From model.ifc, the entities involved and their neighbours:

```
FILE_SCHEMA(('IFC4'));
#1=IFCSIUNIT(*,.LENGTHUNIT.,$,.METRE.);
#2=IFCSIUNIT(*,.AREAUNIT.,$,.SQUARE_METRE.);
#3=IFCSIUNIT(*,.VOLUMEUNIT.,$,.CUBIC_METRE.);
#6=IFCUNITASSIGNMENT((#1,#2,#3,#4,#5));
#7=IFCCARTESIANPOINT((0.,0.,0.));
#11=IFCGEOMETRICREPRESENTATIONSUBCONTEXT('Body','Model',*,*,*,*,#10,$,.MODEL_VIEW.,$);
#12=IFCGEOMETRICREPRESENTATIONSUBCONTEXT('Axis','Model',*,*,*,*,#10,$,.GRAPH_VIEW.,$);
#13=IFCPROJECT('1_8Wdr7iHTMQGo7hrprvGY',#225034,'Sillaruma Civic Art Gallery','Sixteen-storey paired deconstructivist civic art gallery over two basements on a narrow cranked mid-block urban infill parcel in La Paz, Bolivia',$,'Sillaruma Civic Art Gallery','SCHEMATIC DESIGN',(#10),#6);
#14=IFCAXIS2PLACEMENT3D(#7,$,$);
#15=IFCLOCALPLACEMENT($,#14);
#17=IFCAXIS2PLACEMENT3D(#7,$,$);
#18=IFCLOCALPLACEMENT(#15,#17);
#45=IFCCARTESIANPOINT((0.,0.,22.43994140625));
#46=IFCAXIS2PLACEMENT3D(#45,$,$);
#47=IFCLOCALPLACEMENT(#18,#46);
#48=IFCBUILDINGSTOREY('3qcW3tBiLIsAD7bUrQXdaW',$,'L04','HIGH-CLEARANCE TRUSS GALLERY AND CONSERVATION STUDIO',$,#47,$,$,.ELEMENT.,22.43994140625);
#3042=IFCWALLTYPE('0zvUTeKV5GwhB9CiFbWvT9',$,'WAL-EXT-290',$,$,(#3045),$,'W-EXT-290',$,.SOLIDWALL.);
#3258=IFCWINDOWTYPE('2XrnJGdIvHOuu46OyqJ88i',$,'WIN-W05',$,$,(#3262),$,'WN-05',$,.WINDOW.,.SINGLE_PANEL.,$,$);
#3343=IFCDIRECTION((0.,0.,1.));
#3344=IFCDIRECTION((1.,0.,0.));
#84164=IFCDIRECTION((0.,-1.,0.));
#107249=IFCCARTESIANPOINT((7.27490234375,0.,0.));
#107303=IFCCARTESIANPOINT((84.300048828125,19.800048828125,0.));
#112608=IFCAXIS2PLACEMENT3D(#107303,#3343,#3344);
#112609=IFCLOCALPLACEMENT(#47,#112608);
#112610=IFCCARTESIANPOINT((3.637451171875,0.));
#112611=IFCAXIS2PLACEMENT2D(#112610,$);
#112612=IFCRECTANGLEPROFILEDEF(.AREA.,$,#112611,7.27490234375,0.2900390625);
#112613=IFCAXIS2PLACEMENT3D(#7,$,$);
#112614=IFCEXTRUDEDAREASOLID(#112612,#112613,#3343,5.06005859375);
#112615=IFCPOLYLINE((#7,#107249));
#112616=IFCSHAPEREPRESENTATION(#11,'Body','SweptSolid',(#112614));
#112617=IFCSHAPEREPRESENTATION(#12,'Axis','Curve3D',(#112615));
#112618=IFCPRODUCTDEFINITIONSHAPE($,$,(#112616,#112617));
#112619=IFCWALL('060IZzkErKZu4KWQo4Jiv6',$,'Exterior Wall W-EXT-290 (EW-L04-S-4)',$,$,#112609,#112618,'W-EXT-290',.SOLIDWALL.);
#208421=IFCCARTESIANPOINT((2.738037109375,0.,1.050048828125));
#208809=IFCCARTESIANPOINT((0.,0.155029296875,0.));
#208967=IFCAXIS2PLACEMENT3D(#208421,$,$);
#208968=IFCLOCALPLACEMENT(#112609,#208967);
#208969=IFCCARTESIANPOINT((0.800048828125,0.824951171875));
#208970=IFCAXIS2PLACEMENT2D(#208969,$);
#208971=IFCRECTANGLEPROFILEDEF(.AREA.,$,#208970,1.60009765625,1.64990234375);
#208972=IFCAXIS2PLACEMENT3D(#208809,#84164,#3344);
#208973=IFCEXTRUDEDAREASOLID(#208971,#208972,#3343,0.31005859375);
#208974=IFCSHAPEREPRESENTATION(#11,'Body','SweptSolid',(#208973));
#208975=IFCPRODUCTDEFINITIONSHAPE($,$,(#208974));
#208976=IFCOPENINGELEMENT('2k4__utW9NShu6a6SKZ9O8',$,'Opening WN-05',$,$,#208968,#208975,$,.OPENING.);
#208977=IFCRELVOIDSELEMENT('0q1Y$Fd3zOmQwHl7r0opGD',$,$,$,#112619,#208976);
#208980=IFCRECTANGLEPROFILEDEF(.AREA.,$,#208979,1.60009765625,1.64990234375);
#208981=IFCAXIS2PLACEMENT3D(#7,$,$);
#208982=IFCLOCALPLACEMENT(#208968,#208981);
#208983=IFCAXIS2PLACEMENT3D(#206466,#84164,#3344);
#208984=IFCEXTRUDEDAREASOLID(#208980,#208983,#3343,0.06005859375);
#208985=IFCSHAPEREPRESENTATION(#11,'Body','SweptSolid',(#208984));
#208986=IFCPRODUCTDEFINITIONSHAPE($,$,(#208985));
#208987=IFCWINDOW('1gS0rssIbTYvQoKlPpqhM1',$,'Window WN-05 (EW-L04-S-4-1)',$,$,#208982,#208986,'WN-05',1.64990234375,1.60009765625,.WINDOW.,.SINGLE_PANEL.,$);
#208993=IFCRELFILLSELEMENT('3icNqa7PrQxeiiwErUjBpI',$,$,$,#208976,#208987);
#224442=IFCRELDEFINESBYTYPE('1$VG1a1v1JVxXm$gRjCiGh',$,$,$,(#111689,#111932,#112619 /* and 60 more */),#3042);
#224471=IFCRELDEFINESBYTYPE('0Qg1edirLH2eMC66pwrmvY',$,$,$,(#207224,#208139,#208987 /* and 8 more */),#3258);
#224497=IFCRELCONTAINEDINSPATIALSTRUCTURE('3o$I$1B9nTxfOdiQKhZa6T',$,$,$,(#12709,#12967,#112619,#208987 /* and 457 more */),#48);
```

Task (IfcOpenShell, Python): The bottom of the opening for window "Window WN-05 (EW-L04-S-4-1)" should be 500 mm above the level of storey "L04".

```python
import numpy as np
import ifcopenshell
import ifcopenshell.api.geometry
import ifcopenshell.geom
import ifcopenshell.util.element
import ifcopenshell.util.placement
import ifcopenshell.util.shape
import ifcopenshell.util.unit

model = ifcopenshell.open("model.ifc")
unit_scale = ifcopenshell.util.unit.calculate_unit_scale(model)

window = model.by_id(208987)
opening = window.FillsVoids[0].RelatingOpeningElement
storey = ifcopenshell.util.element.get_container(window, ifc_class="IfcBuildingStorey")
level = ifcopenshell.util.placement.get_local_placement(storey.ObjectPlacement)[2, 3]

# The opening's origin need not be at the sill, so measure its lowest point.
shape = ifcopenshell.geom.create_shape(ifcopenshell.geom.settings(), opening)
bottom = ifcopenshell.util.shape.get_shape_bottom_elevation(shape, shape.geometry) / unit_scale
dz = level + 0.5 / unit_scale - bottom

shift = np.array([0.0, 0.0, dz])
# The window is placed relative to its opening, so it follows when the opening moves.
matrix = ifcopenshell.util.placement.get_local_placement(opening.ObjectPlacement)
matrix[:3, 3] += shift
ifcopenshell.api.geometry.edit_object_placement(
    model, product=opening, matrix=matrix, is_si=False, should_transform_children=True
)

print(f"moved by {dz * unit_scale:+.3f} m")

model.write("model_rev.ifc")
```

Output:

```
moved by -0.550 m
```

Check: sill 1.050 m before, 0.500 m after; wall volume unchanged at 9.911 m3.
